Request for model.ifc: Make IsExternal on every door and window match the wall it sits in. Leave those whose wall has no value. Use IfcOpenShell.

First a look at what the model holds.

```python
import ifcopenshell
import ifcopenshell.util.element

model = ifcopenshell.open("model.ifc")
print(model.schema)
seen = {}
for e in model.by_type("IfcDoor") + model.by_type("IfcWindow"):
    if not e.FillsVoids:
        continue
    host = e.FillsVoids[0].RelatingOpeningElement.VoidsElements[0].RelatingBuildingElement
    own = ifcopenshell.util.element.get_pset(e, f"Pset_{e.is_a()[3:].removesuffix('StandardCase')}Common", "IsExternal")
    wall = ifcopenshell.util.element.get_pset(host, "Pset_WallCommon", "IsExternal")
    seen[e.is_a(), own, wall] = seen.get((e.is_a(), own, wall), 0) + 1
for (cls, own, wall), count in sorted(seen.items(), key=str):
    print(count, cls, "IsExternal:", own, "| host wall:", wall)
```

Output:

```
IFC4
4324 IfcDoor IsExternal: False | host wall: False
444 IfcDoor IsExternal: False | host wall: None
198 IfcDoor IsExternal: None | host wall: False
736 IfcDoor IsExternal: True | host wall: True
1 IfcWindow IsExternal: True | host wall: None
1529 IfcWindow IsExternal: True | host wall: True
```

```python
import ifcopenshell
import ifcopenshell.api.pset
import ifcopenshell.util.element

model = ifcopenshell.open("model.ifc")

count = 0
for ifc_class, pset_name in (("IfcDoor", "Pset_DoorCommon"), ("IfcWindow", "Pset_WindowCommon")):
    for e in model.by_type(ifc_class):
        if not e.FillsVoids:
            continue
        host = e.FillsVoids[0].RelatingOpeningElement.VoidsElements[0].RelatingBuildingElement
        external = ifcopenshell.util.element.get_pset(host, "Pset_WallCommon", "IsExternal")
        if external is None or ifcopenshell.util.element.get_pset(e, pset_name, "IsExternal") == external:
            continue
        pset = ifcopenshell.api.pset.add_pset(model, product=e, name=pset_name)
        ifcopenshell.api.pset.edit_pset(model, pset=pset, properties={"IsExternal": external})
        count += 1

print(count, "updated")

model.write("model_v2.ifc")
```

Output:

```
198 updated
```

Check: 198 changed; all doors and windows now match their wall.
